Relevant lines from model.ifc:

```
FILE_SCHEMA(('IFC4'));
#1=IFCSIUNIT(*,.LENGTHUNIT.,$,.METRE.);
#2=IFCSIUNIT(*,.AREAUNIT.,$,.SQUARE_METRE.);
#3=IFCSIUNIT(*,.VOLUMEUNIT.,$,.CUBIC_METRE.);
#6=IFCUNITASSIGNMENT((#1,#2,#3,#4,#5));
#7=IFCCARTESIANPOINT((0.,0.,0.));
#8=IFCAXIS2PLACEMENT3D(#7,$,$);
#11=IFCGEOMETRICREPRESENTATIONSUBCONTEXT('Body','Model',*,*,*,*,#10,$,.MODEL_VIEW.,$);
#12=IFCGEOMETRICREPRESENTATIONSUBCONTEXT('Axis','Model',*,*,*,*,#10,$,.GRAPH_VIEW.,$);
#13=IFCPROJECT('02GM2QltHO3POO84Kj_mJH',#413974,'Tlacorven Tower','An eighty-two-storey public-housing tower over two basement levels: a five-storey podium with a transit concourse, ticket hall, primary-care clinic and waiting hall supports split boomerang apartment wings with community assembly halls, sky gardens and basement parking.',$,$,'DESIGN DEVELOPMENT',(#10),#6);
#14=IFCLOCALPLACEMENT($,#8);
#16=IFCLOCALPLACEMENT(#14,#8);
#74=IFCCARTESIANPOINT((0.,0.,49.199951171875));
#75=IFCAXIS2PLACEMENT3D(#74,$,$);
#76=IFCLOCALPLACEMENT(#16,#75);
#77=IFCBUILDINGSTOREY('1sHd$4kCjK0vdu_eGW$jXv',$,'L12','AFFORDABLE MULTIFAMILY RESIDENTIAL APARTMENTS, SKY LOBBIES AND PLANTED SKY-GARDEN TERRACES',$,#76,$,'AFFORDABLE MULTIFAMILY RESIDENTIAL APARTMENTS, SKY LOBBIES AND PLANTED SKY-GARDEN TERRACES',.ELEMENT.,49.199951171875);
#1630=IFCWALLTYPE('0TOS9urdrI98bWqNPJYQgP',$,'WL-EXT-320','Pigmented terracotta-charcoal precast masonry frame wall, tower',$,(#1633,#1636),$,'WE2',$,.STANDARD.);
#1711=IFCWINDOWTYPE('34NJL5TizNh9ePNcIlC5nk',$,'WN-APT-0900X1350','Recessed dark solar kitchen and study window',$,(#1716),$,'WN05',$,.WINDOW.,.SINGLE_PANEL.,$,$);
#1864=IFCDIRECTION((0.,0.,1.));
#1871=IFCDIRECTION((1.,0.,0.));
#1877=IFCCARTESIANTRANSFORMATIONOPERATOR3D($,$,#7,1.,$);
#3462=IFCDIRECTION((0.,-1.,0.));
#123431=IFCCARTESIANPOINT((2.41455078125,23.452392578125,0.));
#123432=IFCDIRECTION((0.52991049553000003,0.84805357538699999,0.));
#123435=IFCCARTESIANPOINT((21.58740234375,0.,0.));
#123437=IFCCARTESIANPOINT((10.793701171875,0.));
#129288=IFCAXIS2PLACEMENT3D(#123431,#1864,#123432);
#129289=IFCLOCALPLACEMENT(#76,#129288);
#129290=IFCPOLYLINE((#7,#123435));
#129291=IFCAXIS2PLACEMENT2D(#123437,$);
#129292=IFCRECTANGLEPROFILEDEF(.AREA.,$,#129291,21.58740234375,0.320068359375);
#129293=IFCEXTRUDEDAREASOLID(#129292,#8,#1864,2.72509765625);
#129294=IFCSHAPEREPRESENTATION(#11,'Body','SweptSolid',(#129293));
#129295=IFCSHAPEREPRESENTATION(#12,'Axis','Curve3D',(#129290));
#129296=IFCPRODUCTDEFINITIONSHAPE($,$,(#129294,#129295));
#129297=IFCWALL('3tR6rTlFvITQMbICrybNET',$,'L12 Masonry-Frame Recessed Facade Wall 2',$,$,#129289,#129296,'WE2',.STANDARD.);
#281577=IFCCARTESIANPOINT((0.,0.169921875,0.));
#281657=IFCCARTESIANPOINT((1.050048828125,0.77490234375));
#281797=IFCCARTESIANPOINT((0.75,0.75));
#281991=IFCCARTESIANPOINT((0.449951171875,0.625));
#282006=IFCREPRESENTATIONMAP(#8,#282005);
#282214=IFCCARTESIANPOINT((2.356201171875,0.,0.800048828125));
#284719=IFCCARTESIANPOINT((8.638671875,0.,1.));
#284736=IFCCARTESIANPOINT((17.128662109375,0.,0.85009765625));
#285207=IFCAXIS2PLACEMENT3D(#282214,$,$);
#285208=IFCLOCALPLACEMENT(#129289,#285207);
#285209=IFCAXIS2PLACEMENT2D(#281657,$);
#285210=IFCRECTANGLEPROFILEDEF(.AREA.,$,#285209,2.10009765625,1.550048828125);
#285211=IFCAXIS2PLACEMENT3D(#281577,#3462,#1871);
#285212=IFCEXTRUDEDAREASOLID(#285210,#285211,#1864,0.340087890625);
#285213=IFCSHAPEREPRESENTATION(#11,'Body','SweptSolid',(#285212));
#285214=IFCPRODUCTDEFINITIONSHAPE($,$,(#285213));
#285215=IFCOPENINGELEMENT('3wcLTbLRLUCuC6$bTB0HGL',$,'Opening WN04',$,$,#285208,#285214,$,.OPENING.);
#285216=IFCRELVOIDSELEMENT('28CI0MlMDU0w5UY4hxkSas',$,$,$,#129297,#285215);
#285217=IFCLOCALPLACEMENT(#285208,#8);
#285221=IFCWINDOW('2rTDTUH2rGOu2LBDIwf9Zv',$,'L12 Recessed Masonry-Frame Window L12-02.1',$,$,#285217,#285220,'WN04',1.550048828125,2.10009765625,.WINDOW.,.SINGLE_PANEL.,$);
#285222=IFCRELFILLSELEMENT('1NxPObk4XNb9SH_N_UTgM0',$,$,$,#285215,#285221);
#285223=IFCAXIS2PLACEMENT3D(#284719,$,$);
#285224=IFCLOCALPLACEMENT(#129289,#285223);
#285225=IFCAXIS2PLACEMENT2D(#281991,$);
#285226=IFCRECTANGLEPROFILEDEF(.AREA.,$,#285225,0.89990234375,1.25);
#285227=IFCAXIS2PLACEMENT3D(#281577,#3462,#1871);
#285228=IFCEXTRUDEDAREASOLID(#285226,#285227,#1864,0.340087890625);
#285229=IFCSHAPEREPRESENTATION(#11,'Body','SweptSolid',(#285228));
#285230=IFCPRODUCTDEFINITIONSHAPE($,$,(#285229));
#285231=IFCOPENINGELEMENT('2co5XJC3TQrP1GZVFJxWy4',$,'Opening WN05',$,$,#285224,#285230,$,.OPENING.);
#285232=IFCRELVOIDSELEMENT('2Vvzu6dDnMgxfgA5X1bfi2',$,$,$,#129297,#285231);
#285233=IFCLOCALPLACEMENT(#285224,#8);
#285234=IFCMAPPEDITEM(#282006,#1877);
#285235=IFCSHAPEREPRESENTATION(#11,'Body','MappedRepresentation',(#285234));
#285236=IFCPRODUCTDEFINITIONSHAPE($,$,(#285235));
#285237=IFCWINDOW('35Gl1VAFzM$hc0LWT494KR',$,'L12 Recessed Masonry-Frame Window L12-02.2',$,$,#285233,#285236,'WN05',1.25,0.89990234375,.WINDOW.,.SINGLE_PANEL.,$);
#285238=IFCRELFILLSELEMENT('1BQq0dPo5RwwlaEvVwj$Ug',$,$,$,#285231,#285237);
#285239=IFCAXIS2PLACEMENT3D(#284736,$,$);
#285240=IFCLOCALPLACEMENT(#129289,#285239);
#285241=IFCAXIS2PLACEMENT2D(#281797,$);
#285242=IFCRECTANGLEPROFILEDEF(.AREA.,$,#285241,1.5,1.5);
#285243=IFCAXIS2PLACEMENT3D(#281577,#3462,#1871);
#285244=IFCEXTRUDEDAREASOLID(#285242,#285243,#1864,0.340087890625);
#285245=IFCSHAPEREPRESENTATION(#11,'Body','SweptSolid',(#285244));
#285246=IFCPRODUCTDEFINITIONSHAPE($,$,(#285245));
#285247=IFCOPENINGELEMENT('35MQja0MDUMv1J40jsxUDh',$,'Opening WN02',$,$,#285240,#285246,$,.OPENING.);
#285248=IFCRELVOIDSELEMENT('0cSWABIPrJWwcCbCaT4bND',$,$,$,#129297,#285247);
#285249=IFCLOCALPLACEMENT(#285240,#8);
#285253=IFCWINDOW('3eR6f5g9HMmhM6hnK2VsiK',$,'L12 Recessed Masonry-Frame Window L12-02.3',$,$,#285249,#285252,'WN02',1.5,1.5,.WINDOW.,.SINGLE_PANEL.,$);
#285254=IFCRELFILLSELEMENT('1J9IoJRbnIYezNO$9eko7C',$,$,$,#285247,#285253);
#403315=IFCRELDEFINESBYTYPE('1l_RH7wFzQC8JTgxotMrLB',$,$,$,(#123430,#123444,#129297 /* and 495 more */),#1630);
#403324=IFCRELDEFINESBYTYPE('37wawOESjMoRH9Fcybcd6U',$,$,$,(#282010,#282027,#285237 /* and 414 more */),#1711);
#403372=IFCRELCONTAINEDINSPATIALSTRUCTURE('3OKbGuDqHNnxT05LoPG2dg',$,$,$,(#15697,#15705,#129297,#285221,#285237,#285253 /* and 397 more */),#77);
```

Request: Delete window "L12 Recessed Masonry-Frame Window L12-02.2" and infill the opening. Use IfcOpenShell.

```python
import ifcopenshell
import ifcopenshell.api.feature
import ifcopenshell.api.root
import ifcopenshell.geom
import ifcopenshell.util.shape

model = ifcopenshell.open("model.ifc")
settings = ifcopenshell.geom.settings()


def volume(element):
    """Net volume in cubic metres, openings subtracted."""
    shape = ifcopenshell.geom.create_shape(settings, element)
    return ifcopenshell.util.shape.get_volume(shape.geometry)


window = model.by_guid("35Gl1VAFzM$hc0LWT494KR")
opening = window.FillsVoids[0].RelatingOpeningElement
wall = opening.VoidsElements[0].RelatingBuildingElement
before = volume(wall)

ifcopenshell.api.root.remove_product(model, product=window)
ifcopenshell.api.feature.remove_feature(model, feature=opening)

after = volume(wall)

print(f"wall volume {before:.3f} -> {after:.3f} m3")

model.write("model_updated.ifc")
```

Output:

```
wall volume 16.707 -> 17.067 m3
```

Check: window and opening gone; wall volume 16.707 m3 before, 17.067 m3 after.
